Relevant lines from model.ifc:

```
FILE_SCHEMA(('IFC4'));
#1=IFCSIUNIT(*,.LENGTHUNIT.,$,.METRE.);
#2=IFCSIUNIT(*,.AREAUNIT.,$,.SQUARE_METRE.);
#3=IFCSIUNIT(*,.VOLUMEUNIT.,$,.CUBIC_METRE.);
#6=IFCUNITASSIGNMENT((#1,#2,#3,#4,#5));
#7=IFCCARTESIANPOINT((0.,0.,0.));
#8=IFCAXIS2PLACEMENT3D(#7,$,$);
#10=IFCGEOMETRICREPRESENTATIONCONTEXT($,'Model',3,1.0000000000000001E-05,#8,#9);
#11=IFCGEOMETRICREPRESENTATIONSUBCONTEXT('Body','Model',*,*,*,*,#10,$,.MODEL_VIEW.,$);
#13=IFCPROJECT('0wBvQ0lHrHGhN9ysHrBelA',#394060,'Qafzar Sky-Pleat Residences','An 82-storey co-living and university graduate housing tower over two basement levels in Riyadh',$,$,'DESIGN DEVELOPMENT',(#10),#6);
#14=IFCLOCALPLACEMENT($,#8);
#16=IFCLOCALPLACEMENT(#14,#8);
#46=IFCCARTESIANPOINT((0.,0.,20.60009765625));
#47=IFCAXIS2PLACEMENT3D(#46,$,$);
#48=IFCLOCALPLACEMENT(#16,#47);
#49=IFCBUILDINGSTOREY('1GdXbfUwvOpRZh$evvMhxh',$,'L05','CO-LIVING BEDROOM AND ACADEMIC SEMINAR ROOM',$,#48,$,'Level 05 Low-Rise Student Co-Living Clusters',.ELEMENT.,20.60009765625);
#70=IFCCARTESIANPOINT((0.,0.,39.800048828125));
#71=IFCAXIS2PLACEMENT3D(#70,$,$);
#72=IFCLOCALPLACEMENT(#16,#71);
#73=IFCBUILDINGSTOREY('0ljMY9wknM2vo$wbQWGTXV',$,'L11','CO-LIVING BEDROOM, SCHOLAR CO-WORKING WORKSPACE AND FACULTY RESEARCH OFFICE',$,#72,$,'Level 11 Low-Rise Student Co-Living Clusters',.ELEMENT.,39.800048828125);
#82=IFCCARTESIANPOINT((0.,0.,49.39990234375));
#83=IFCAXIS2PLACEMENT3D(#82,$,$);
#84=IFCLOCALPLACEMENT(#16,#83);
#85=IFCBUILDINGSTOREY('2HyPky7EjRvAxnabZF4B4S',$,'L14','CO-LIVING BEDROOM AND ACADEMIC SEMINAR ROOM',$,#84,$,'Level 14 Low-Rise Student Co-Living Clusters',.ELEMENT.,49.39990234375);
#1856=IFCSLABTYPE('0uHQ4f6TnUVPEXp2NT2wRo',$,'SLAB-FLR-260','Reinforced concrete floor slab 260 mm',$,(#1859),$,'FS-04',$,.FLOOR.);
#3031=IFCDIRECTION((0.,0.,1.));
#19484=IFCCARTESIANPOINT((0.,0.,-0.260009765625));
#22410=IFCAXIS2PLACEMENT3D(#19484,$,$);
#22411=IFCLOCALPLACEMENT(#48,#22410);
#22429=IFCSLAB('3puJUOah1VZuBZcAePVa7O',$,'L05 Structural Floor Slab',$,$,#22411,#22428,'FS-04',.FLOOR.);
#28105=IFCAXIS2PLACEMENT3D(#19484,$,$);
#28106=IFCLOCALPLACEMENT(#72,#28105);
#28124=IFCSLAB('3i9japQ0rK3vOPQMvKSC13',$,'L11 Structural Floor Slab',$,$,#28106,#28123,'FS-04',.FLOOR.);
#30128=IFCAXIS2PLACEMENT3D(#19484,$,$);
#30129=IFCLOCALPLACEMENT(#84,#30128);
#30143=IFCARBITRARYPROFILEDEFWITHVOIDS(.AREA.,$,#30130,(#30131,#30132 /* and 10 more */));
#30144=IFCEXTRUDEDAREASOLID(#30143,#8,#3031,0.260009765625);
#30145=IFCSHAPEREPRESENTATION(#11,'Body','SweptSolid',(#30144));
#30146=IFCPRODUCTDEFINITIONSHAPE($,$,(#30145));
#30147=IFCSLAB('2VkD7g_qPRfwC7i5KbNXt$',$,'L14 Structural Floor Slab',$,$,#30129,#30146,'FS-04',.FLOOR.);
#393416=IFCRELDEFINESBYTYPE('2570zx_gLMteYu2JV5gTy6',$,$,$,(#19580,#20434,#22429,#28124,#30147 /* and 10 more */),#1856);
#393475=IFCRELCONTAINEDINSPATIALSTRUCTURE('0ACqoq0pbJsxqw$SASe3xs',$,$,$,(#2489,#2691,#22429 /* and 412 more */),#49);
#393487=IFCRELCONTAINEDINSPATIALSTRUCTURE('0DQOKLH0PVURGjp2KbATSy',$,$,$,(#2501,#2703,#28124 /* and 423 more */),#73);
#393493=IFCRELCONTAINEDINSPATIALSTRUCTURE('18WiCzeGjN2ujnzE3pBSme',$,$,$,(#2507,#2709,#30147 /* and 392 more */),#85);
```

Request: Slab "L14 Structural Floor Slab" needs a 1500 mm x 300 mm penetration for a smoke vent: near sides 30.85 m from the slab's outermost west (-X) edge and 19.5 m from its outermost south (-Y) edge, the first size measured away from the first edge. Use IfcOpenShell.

```python
import numpy as np
import ifcopenshell
import ifcopenshell.api.feature
import ifcopenshell.api.geometry
import ifcopenshell.api.root
import ifcopenshell.geom
import ifcopenshell.util.placement
import ifcopenshell.util.representation
import ifcopenshell.util.shape
import ifcopenshell.util.unit

model = ifcopenshell.open("model.ifc")
unit_scale = ifcopenshell.util.unit.calculate_unit_scale(model)
settings = ifcopenshell.geom.settings()


def volume(element):
    """Net volume in cubic metres, openings subtracted."""
    shape = ifcopenshell.geom.create_shape(settings, element)
    return ifcopenshell.util.shape.get_volume(shape.geometry)


slab = model.by_guid("2VkD7g_qPRfwC7i5KbNXt$")
before = volume(slab)

# Extent in the slab's own axes, in metres. The edges named are its -X and -Y sides.
slab_shape = ifcopenshell.geom.create_shape(settings, slab)
vertices = ifcopenshell.util.shape.get_vertices(slab_shape.geometry)
x_min, y_min, bottom = vertices.min(axis=0)
top = vertices[:, 2].max()

opening = ifcopenshell.api.root.create_entity(model, ifc_class="IfcOpeningElement", name="Smoke vent opening", predefined_type="OPENING")
context = ifcopenshell.util.representation.get_context(model, "Model", "Body", "MODEL_VIEW")
width, depth = 1.5, 0.3
outline = [(0.0, 0.0), (width, 0.0), (width, depth), (0.0, depth), (0.0, 0.0)]
# Overshoot both faces by 50 mm so the cut is clean.
shape = ifcopenshell.api.geometry.add_slab_representation(
    model, context=context, depth=top - bottom + 0.1, polyline=outline
)
ifcopenshell.api.geometry.assign_representation(model, product=opening, representation=shape)

matrix = ifcopenshell.util.placement.get_local_placement(slab.ObjectPlacement)
matrix[:, 3] = matrix @ np.append(np.array([x_min + 30.85, y_min + 19.5, bottom - 0.05]) / unit_scale, 1.0)
ifcopenshell.api.geometry.edit_object_placement(model, product=opening, matrix=matrix, is_si=False)
ifcopenshell.api.feature.add_feature(model, feature=opening, element=slab)

after = volume(slab)

print(f"slab volume {before:.3f} -> {after:.3f} m3")

model.write("model_rev.ifc")
```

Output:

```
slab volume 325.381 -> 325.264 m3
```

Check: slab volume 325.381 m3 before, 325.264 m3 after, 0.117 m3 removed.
